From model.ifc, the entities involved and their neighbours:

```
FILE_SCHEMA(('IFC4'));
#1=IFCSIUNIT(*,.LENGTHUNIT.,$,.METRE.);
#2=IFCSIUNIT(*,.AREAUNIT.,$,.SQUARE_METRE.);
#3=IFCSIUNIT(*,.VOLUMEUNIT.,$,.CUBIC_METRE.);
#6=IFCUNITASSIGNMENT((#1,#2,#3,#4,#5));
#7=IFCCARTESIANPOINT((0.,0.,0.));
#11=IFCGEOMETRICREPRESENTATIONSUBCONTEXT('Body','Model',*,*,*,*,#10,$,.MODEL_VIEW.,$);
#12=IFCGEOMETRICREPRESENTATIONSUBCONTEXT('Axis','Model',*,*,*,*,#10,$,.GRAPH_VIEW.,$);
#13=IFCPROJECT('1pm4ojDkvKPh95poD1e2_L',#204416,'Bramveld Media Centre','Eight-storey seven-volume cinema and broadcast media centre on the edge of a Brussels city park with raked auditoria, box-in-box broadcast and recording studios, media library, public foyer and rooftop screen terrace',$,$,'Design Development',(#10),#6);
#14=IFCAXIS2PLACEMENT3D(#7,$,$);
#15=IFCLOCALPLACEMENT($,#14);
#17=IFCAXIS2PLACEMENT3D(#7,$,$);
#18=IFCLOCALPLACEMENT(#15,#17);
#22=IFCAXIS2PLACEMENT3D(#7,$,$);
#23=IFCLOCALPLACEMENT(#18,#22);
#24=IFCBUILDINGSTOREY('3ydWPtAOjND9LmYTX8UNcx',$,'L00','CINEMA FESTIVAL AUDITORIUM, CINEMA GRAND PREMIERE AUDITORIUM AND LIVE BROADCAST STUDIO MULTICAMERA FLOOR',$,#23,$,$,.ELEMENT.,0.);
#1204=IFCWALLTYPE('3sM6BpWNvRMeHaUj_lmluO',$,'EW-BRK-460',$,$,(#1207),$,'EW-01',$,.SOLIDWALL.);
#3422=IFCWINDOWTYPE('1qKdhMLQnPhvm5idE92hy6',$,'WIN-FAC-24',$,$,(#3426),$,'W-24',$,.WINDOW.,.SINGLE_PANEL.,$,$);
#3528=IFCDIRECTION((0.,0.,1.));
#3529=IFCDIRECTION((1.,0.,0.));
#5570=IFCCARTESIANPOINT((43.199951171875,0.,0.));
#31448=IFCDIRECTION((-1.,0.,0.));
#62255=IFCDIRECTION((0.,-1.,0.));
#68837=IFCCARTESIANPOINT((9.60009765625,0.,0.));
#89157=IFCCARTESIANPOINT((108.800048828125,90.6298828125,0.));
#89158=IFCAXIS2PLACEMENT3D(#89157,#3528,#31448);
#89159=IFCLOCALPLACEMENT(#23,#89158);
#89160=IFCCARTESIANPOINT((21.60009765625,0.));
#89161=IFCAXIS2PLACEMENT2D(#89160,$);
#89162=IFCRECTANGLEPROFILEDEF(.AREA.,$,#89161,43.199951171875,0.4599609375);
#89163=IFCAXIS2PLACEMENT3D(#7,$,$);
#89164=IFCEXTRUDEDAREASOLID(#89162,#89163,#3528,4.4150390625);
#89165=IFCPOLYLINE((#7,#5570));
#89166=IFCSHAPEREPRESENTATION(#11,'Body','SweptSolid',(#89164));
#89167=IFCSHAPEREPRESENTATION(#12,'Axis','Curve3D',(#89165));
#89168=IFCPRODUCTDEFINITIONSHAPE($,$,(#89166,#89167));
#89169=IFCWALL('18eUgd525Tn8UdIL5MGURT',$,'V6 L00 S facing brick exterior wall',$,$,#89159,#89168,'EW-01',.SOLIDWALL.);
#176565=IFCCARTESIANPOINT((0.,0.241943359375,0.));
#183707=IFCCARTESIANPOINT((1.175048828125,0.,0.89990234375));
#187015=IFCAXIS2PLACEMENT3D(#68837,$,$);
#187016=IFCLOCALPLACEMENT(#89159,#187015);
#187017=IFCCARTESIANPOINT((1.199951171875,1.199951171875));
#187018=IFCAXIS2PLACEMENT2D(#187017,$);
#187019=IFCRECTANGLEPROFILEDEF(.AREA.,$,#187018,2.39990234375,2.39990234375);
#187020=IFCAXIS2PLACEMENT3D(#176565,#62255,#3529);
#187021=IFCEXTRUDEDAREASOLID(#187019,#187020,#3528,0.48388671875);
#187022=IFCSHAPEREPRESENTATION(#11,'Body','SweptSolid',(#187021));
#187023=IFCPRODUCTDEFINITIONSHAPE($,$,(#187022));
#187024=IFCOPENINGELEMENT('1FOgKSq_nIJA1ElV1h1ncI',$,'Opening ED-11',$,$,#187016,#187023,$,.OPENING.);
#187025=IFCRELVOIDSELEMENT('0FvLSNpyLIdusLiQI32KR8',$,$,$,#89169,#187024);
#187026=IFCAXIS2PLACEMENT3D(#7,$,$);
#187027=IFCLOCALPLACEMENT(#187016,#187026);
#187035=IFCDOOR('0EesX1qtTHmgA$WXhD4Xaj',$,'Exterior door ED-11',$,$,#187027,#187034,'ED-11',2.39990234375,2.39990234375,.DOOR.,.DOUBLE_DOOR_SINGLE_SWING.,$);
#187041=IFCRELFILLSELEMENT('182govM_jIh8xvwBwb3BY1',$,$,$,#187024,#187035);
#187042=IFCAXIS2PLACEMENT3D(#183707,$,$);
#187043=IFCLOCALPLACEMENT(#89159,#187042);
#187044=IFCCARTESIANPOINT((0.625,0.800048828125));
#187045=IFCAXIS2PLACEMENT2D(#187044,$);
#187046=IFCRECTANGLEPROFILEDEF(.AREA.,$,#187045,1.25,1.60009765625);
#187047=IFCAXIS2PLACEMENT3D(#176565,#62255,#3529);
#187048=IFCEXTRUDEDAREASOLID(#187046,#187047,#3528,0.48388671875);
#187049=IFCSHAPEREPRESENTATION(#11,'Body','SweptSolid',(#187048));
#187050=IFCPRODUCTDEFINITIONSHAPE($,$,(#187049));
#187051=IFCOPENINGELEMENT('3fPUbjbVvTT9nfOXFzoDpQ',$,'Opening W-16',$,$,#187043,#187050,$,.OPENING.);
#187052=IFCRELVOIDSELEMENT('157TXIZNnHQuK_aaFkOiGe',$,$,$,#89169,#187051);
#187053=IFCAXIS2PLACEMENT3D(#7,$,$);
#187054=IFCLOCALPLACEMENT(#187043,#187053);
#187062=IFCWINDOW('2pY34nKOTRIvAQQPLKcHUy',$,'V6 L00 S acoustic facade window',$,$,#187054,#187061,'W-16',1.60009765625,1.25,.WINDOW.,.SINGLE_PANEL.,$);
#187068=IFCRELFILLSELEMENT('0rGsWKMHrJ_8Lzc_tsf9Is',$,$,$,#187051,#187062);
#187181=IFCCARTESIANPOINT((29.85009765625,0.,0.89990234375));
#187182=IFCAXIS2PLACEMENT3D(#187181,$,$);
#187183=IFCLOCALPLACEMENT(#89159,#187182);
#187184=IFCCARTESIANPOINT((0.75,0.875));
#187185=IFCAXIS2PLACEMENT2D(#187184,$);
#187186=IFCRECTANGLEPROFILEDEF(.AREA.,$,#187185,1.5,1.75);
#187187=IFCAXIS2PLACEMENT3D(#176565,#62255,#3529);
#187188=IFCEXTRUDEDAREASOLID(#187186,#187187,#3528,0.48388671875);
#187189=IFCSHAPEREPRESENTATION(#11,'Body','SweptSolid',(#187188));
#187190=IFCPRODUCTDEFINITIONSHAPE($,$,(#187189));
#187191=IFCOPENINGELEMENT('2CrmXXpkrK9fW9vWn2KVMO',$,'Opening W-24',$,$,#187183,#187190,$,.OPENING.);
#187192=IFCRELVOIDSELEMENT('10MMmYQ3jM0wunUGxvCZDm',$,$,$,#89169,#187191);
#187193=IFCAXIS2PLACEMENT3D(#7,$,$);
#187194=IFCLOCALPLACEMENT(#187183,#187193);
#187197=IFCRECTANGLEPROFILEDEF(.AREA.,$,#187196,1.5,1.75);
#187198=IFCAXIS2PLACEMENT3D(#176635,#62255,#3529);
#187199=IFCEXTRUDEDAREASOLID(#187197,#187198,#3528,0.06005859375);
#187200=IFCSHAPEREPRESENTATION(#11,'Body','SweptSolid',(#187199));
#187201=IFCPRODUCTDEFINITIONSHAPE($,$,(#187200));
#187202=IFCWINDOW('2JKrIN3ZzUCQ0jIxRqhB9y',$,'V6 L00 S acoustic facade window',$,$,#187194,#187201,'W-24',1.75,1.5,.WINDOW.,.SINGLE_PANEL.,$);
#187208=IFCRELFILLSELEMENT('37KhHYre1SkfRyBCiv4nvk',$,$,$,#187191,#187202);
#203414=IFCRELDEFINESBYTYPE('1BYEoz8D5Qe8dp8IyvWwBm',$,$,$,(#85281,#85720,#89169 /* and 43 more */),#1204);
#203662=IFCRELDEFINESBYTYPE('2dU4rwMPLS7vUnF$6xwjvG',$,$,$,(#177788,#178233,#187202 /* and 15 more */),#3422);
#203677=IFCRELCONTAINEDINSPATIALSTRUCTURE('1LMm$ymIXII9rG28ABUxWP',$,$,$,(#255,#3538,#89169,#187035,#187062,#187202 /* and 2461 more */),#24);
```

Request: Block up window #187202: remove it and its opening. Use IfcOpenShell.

```python
import ifcopenshell
import ifcopenshell.api.feature
import ifcopenshell.api.root
import ifcopenshell.geom
import ifcopenshell.util.shape

model = ifcopenshell.open("model.ifc")
settings = ifcopenshell.geom.settings()


def volume(element):
    """Net volume in cubic metres, openings subtracted."""
    shape = ifcopenshell.geom.create_shape(settings, element)
    return ifcopenshell.util.shape.get_volume(shape.geometry)


window = model.by_guid("2JKrIN3ZzUCQ0jIxRqhB9y")
opening = window.FillsVoids[0].RelatingOpeningElement
wall = opening.VoidsElements[0].RelatingBuildingElement
before = volume(wall)

ifcopenshell.api.root.remove_product(model, product=window)
ifcopenshell.api.feature.remove_feature(model, feature=opening)

after = volume(wall)

print(f"wall volume {before:.3f} -> {after:.3f} m3")

model.write("model_edited.ifc")
```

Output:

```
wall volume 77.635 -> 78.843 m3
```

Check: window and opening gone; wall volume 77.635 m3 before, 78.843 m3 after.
